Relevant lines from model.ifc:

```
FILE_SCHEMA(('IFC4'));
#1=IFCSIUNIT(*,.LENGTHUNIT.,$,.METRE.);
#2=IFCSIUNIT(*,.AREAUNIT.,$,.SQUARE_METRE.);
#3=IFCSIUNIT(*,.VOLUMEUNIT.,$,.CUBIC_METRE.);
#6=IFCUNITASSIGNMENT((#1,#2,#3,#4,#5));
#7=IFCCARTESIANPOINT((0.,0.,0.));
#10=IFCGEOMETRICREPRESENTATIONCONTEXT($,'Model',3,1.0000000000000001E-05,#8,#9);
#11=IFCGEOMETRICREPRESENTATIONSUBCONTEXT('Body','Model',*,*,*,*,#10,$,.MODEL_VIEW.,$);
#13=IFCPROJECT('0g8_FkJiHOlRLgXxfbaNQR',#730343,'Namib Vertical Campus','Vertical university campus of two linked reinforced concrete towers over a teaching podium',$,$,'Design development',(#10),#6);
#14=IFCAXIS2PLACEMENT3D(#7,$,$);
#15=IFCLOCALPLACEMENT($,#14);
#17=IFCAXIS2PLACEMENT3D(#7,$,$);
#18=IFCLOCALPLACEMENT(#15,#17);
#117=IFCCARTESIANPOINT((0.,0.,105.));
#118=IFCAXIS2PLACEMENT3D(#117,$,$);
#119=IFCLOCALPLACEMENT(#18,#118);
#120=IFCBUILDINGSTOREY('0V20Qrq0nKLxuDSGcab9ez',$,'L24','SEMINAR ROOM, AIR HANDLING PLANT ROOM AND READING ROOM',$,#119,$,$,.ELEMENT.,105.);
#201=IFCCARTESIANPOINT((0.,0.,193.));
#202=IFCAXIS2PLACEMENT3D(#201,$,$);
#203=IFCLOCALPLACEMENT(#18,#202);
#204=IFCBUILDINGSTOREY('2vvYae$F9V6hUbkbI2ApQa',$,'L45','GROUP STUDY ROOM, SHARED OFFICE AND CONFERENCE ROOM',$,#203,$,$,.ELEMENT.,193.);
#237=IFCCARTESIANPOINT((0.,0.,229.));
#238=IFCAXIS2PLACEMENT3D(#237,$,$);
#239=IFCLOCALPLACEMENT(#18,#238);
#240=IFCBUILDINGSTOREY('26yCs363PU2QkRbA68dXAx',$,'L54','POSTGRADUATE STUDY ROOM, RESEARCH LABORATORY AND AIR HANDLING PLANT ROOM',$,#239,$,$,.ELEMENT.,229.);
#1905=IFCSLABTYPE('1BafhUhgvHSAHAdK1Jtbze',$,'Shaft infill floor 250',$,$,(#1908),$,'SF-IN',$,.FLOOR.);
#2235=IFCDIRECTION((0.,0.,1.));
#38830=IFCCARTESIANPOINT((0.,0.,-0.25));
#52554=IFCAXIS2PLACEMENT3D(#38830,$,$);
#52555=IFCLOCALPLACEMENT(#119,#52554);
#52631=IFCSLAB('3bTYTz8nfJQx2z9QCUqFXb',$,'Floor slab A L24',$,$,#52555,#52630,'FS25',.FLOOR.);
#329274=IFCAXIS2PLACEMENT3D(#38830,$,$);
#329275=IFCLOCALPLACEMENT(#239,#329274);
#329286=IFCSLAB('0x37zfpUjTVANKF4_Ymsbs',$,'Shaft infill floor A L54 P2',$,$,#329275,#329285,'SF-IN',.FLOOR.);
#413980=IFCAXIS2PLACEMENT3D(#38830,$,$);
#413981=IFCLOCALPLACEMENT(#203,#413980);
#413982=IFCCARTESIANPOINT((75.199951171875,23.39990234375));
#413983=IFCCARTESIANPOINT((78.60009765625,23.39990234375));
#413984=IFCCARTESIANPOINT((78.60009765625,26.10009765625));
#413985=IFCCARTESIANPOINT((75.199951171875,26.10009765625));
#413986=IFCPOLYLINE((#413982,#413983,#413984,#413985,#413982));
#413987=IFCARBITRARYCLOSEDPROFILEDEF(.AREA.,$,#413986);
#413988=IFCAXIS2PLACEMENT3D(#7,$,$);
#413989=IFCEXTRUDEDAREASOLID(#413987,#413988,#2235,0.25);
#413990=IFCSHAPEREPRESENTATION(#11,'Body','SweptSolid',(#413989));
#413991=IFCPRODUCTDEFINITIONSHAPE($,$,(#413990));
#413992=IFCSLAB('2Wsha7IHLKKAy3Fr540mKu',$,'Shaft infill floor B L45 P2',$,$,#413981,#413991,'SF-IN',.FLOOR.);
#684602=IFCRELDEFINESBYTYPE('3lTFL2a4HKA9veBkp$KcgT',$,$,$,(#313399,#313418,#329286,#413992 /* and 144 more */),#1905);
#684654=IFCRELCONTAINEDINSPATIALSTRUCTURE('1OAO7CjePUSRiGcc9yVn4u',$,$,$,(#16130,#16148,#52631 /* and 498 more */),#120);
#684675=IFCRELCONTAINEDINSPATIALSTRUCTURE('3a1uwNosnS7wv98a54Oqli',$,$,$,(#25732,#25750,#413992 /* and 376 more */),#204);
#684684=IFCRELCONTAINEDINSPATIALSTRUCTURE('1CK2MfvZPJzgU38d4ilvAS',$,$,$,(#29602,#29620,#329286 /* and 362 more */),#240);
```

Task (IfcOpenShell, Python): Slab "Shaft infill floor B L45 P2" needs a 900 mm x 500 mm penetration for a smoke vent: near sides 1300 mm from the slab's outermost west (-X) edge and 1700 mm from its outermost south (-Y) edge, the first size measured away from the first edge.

```python
import numpy as np
import ifcopenshell
import ifcopenshell.api.feature
import ifcopenshell.api.geometry
import ifcopenshell.api.root
import ifcopenshell.geom
import ifcopenshell.util.placement
import ifcopenshell.util.representation
import ifcopenshell.util.shape
import ifcopenshell.util.unit

model = ifcopenshell.open("model.ifc")
unit_scale = ifcopenshell.util.unit.calculate_unit_scale(model)
settings = ifcopenshell.geom.settings()


def volume(element):
    """Net volume in cubic metres, openings subtracted."""
    shape = ifcopenshell.geom.create_shape(settings, element)
    return ifcopenshell.util.shape.get_volume(shape.geometry)


slab = model.by_guid("2Wsha7IHLKKAy3Fr540mKu")
before = volume(slab)

# Extent in the slab's own axes, in metres. The edges named are its -X and -Y sides.
slab_shape = ifcopenshell.geom.create_shape(settings, slab)
vertices = ifcopenshell.util.shape.get_vertices(slab_shape.geometry)
x_min, y_min, bottom = vertices.min(axis=0)
top = vertices[:, 2].max()

opening = ifcopenshell.api.root.create_entity(model, ifc_class="IfcOpeningElement", name="Smoke vent opening", predefined_type="OPENING")
context = ifcopenshell.util.representation.get_context(model, "Model", "Body", "MODEL_VIEW")
width, depth = 0.9, 0.5
outline = [(0.0, 0.0), (width, 0.0), (width, depth), (0.0, depth), (0.0, 0.0)]
# Overshoot both faces by 50 mm so the cut is clean.
shape = ifcopenshell.api.geometry.add_slab_representation(
    model, context=context, depth=top - bottom + 0.1, polyline=outline
)
ifcopenshell.api.geometry.assign_representation(model, product=opening, representation=shape)

matrix = ifcopenshell.util.placement.get_local_placement(slab.ObjectPlacement)
matrix[:, 3] = matrix @ np.append(np.array([x_min + 1.3, y_min + 1.7, bottom - 0.05]) / unit_scale, 1.0)
ifcopenshell.api.geometry.edit_object_placement(model, product=opening, matrix=matrix, is_si=False)
ifcopenshell.api.feature.add_feature(model, feature=opening, element=slab)

after = volume(slab)

print(f"slab volume {before:.3f} -> {after:.3f} m3")

model.write("model_rev.ifc")
```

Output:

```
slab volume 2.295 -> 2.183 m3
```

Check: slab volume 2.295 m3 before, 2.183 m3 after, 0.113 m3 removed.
